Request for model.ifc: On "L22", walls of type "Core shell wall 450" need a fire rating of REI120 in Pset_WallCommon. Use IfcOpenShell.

First a look at what the model holds.

```python
import ifcopenshell
import ifcopenshell.util.element

model = ifcopenshell.open("model.ifc")
print(model.schema)
storey = next(s for s in model.by_type("IfcBuildingStorey") if s.Name == "L22")
walls = [e for e in ifcopenshell.util.element.get_decomposition(storey) if e.is_a("IfcWall")]
seen = {}
for e in walls:
    element_type = ifcopenshell.util.element.get_type(e)
    key = (element_type.Name if element_type != e and element_type else None, ifcopenshell.util.element.get_pset(e, "Pset_WallCommon", "FireRating"))
    seen[key] = seen.get(key, 0) + 1
for (name, value), count in sorted(seen.items(), key=str):
    print(count, "x", name, "|", value)
```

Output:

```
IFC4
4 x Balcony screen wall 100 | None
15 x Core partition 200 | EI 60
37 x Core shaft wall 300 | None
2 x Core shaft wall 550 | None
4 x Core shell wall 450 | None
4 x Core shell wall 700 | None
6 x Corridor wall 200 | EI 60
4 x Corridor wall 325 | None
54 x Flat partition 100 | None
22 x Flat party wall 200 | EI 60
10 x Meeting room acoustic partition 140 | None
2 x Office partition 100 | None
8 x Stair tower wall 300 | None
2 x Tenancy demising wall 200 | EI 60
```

```python
import ifcopenshell
import ifcopenshell.api.pset
import ifcopenshell.util.element

model = ifcopenshell.open("model.ifc")

storey = next(s for s in model.by_type("IfcBuildingStorey") if s.Name == "L22")
walls = [e for e in ifcopenshell.util.element.get_decomposition(storey) if e.is_a("IfcWall")]

count = 0
for e in walls:
    element_type = ifcopenshell.util.element.get_type(e)
    if element_type in (None, e) or element_type.Name != "Core shell wall 450":
        continue
    found = ifcopenshell.util.element.get_pset(e, "Pset_WallCommon", should_inherit=False)
    if found:
        pset = model.by_id(found["id"])
        if len(ifcopenshell.util.element.get_elements_by_pset(pset)) > 1:
            pset = ifcopenshell.api.pset.unshare_pset(model, products=[e], pset=pset)[0]
    else:
        pset = ifcopenshell.api.pset.add_pset(model, product=e, name="Pset_WallCommon")
    ifcopenshell.api.pset.edit_pset(model, pset=pset, properties={"FireRating": "REI120"})
    count += 1

print(count, "walls updated")

model.write("model_edited.ifc")
```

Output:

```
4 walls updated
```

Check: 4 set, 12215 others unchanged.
